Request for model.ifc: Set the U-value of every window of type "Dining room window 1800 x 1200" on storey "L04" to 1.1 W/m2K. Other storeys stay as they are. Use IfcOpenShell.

First a look at what the model holds.

```python
import ifcopenshell
import ifcopenshell.util.element

model = ifcopenshell.open("model.ifc")
print(model.schema)
storey = next(s for s in model.by_type("IfcBuildingStorey") if s.Name == "L04")
windows = [e for e in ifcopenshell.util.element.get_decomposition(storey) if e.is_a("IfcWindow")]
seen = {}
for e in windows:
    element_type = ifcopenshell.util.element.get_type(e)
    key = (element_type.Name if element_type != e and element_type else None, ifcopenshell.util.element.get_pset(e, "Pset_WindowCommon", "ThermalTransmittance"))
    seen[key] = seen.get(key, 0) + 1
for (name, value), count in sorted(seen.items(), key=str):
    print(count, "x", name, "|", value)
```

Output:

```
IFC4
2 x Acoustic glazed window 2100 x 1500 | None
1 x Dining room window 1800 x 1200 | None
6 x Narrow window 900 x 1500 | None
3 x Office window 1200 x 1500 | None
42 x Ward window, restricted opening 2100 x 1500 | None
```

```python
import ifcopenshell
import ifcopenshell.api.pset
import ifcopenshell.util.element

model = ifcopenshell.open("model.ifc")

storey = next(s for s in model.by_type("IfcBuildingStorey") if s.Name == "L04")
windows = [e for e in ifcopenshell.util.element.get_decomposition(storey) if e.is_a("IfcWindow")]

count = 0
for e in windows:
    element_type = ifcopenshell.util.element.get_type(e)
    if element_type in (None, e) or element_type.Name != "Dining room window 1800 x 1200":
        continue
    # add_pset returns the element's existing set when there is one.
    pset = ifcopenshell.api.pset.add_pset(model, product=e, name="Pset_WindowCommon")
    ifcopenshell.api.pset.edit_pset(model, pset=pset, properties={"ThermalTransmittance": 1.1})
    count += 1

print(count, "windows updated")

model.write("model_updated.ifc")
```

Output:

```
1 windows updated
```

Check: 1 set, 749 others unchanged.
